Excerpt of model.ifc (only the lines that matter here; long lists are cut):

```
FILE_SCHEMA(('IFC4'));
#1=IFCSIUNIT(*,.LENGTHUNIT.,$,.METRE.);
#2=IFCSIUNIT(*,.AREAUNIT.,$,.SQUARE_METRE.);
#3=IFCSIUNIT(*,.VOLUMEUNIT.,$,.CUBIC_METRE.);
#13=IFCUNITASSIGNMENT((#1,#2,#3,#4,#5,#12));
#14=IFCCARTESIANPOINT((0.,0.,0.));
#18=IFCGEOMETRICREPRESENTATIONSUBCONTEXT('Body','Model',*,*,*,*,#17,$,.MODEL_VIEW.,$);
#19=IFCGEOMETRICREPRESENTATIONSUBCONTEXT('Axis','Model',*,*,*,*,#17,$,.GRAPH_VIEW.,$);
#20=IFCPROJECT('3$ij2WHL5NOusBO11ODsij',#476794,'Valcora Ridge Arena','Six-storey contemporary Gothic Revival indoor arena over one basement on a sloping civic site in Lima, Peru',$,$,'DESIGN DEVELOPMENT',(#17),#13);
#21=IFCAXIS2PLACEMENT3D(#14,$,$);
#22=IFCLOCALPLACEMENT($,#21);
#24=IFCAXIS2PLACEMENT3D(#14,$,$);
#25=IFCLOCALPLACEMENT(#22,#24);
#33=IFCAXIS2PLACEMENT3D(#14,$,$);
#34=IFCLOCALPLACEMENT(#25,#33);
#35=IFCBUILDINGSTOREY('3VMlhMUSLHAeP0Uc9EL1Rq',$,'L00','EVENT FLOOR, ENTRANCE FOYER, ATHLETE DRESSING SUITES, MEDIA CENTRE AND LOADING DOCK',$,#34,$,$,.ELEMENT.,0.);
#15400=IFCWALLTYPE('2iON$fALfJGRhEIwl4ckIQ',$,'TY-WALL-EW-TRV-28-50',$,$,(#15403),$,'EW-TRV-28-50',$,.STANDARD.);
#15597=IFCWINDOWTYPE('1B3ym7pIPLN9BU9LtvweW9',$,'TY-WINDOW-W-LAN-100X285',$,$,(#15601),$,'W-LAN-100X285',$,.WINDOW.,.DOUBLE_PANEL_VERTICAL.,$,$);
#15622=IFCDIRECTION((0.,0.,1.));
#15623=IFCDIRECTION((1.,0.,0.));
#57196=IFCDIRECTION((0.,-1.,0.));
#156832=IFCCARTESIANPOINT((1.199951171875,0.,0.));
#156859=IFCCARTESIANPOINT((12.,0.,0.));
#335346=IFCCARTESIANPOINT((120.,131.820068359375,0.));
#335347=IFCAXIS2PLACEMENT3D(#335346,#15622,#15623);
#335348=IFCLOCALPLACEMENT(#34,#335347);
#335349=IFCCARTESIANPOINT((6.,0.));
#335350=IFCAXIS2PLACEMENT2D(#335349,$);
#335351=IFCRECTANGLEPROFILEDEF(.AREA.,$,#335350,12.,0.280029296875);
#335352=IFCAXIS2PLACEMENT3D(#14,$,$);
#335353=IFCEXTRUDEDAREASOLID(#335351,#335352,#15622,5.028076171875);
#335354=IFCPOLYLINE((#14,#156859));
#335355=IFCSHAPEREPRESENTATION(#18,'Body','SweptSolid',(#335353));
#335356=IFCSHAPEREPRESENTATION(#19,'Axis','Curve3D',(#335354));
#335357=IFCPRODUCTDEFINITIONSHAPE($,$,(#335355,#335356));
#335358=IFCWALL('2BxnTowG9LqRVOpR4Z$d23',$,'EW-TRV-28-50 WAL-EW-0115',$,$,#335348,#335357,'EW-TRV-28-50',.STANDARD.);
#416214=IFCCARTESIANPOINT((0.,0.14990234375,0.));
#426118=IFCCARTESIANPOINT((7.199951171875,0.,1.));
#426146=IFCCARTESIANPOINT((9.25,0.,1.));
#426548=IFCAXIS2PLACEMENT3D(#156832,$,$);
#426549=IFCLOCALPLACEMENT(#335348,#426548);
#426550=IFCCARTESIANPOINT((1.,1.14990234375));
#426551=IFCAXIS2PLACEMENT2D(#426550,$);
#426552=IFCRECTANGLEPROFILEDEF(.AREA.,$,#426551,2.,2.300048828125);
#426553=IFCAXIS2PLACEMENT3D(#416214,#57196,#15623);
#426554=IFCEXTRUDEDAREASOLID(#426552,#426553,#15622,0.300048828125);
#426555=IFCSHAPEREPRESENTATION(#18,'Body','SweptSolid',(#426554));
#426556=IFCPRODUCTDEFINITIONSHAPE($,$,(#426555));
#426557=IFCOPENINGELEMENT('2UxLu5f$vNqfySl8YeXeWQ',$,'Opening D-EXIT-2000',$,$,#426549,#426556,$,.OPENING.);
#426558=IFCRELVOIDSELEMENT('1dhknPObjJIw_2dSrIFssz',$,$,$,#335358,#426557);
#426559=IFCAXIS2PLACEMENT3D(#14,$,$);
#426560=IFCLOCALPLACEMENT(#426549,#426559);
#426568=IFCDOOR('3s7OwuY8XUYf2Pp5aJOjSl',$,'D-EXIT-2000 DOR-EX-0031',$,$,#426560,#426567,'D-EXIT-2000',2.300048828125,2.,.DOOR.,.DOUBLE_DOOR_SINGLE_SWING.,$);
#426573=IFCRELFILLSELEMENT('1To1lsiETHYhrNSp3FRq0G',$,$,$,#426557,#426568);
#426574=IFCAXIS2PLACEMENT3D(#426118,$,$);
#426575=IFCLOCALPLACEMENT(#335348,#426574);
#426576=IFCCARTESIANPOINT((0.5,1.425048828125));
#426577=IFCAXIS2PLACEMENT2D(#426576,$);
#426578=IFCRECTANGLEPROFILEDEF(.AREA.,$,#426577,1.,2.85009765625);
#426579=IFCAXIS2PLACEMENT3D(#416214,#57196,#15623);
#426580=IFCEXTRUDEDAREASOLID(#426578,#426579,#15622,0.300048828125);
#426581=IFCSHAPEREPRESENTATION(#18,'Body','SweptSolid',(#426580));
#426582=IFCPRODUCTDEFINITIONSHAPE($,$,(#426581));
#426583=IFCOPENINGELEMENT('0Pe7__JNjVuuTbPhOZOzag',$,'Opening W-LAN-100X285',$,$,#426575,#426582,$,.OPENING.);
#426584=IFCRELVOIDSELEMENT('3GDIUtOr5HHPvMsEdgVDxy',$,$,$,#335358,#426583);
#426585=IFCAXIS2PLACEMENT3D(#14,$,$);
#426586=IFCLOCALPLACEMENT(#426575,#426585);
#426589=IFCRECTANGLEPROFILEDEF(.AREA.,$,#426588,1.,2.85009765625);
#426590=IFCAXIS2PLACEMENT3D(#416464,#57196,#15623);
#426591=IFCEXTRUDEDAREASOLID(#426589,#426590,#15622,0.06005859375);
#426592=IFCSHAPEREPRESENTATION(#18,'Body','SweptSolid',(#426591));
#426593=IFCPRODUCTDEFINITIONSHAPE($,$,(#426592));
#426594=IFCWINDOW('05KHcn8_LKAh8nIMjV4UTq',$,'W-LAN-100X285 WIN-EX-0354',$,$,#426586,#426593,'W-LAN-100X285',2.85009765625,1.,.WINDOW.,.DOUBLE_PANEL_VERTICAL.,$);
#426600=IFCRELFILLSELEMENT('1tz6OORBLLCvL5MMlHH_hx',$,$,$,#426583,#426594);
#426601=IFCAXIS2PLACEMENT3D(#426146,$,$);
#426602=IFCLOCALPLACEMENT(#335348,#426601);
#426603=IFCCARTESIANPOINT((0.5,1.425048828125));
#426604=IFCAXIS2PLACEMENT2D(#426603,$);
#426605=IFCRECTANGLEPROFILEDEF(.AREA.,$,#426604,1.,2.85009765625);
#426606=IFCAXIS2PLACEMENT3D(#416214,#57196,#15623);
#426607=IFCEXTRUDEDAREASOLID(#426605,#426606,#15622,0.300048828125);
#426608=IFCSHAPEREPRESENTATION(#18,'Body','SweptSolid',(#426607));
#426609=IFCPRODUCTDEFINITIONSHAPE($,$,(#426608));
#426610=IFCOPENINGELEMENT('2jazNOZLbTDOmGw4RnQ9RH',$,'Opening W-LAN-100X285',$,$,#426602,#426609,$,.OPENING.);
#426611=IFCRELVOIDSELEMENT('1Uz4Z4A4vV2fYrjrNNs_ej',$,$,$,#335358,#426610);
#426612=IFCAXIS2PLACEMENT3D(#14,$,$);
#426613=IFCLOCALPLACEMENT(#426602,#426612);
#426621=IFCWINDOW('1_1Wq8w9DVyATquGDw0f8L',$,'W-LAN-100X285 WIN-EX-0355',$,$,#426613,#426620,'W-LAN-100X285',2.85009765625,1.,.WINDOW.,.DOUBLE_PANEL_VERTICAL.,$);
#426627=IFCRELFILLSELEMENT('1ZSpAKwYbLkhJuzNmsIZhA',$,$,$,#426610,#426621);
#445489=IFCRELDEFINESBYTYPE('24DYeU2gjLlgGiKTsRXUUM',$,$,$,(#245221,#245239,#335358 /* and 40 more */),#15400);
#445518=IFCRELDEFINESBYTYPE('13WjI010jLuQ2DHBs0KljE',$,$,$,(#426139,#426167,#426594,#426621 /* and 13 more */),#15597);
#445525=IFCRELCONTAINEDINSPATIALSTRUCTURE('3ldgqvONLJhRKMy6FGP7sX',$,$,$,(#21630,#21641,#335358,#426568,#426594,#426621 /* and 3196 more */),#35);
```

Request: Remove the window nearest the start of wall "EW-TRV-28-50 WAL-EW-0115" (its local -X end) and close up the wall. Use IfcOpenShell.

```python
import ifcopenshell
import ifcopenshell.api.feature
import ifcopenshell.api.root
import ifcopenshell.geom
import ifcopenshell.util.shape

model = ifcopenshell.open("model.ifc")
settings = ifcopenshell.geom.settings()


def volume(element):
    """Net volume in cubic metres, openings subtracted."""
    shape = ifcopenshell.geom.create_shape(settings, element)
    return ifcopenshell.util.shape.get_volume(shape.geometry)


window = model.by_guid("05KHcn8_LKAh8nIMjV4UTq")
opening = window.FillsVoids[0].RelatingOpeningElement
wall = opening.VoidsElements[0].RelatingBuildingElement
before = volume(wall)

ifcopenshell.api.root.remove_product(model, product=window)
ifcopenshell.api.feature.remove_feature(model, feature=opening)

after = volume(wall)

print(f"wall volume {before:.3f} -> {after:.3f} m3")

model.write("model_rev.ifc")
```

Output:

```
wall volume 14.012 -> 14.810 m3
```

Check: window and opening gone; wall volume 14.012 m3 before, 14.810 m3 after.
